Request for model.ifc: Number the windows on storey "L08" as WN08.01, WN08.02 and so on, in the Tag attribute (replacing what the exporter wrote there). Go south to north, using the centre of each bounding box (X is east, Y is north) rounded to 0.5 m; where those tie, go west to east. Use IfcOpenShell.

First a look at what the model holds.

```python
import ifcopenshell
import ifcopenshell.util.element
import ifcopenshell.util.placement

model = ifcopenshell.open("model.ifc")
print(model.schema)
storey = next(s for s in model.by_type("IfcBuildingStorey") if s.Name == "L08")
windows = [e for e in ifcopenshell.util.element.get_decomposition(storey) if e.is_a("IfcWindow")]
for e in sorted(windows, key=lambda e: e.id()):
    origin = ifcopenshell.util.placement.get_local_placement(e.ObjectPlacement)[:3, 3]
    print(e.id(), e.Tag, e.Name, origin.round(2) + 0.0, sep=" | ")
```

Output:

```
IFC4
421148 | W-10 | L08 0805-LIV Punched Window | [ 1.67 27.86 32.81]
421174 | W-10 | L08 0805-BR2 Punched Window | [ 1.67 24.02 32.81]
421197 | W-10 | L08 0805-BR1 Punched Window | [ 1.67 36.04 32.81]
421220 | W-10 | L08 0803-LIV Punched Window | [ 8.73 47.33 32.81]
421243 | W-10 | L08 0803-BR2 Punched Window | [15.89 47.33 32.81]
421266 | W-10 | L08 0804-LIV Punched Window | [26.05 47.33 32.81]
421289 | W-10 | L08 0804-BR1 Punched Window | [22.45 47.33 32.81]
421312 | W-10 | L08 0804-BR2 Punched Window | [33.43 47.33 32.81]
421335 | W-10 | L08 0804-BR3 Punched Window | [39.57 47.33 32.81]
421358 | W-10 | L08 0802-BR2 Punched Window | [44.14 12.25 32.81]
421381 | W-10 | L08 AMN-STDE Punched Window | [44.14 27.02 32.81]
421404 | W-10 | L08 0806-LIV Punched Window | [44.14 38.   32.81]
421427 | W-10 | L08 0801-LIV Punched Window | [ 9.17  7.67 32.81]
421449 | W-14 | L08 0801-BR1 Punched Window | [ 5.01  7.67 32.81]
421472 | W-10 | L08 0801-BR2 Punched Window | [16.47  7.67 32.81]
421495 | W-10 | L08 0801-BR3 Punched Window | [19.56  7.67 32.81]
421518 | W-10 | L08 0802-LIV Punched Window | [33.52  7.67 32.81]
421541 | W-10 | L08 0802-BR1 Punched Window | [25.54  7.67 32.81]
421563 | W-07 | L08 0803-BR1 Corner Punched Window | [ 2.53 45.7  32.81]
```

```python
import ifcopenshell
import ifcopenshell.geom
import ifcopenshell.util.element
import ifcopenshell.util.shape

model = ifcopenshell.open("model.ifc")
settings = ifcopenshell.geom.settings()
settings.set("use-world-coords", True)


def centre(element):
    shape = ifcopenshell.geom.create_shape(settings, element)
    return ifcopenshell.util.shape.get_bbox_centroid(shape.geometry)


storey = next(s for s in model.by_type("IfcBuildingStorey") if s.Name == "L08")
windows = [e for e in ifcopenshell.util.element.get_decomposition(storey) if e.is_a("IfcWindow")]

# Insertion points can sit at a corner or the storey origin, so sort by the geometry (in metres).
centres = {e: centre(e) for e in windows}
windows.sort(key=lambda e: (round(centres[e][1] / 0.5), centres[e][0]))

for i, e in enumerate(windows, start=1):
    number = f"WN08.{i:02d}"
    e.Tag = number
    print(e.id(), number)

model.write("model_updated.ifc")
```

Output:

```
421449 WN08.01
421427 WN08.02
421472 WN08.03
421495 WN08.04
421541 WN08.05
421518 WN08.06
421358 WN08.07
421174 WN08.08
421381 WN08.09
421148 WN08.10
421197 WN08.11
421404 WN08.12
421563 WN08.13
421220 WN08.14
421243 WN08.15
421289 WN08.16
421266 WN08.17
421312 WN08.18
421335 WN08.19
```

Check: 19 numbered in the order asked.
